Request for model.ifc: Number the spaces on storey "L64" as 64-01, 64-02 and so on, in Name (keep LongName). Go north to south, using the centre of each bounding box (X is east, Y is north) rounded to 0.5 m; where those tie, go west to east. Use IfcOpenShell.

First a look at what the model holds.

```python
import ifcopenshell
import ifcopenshell.util.element
import ifcopenshell.util.placement

model = ifcopenshell.open("model.ifc")
print(model.schema)
storey = next(s for s in model.by_type("IfcBuildingStorey") if s.Name == "L64")
spaces = [e for e in ifcopenshell.util.element.get_decomposition(storey) if e.is_a("IfcSpace")]
for e in sorted(spaces, key=lambda e: e.id()):
    origin = ifcopenshell.util.placement.get_local_placement(e.ObjectPlacement)[:3, 3]
    print(e.id(), e.Name, e.LongName, origin.round(2) + 0.0, sep=" | ")
```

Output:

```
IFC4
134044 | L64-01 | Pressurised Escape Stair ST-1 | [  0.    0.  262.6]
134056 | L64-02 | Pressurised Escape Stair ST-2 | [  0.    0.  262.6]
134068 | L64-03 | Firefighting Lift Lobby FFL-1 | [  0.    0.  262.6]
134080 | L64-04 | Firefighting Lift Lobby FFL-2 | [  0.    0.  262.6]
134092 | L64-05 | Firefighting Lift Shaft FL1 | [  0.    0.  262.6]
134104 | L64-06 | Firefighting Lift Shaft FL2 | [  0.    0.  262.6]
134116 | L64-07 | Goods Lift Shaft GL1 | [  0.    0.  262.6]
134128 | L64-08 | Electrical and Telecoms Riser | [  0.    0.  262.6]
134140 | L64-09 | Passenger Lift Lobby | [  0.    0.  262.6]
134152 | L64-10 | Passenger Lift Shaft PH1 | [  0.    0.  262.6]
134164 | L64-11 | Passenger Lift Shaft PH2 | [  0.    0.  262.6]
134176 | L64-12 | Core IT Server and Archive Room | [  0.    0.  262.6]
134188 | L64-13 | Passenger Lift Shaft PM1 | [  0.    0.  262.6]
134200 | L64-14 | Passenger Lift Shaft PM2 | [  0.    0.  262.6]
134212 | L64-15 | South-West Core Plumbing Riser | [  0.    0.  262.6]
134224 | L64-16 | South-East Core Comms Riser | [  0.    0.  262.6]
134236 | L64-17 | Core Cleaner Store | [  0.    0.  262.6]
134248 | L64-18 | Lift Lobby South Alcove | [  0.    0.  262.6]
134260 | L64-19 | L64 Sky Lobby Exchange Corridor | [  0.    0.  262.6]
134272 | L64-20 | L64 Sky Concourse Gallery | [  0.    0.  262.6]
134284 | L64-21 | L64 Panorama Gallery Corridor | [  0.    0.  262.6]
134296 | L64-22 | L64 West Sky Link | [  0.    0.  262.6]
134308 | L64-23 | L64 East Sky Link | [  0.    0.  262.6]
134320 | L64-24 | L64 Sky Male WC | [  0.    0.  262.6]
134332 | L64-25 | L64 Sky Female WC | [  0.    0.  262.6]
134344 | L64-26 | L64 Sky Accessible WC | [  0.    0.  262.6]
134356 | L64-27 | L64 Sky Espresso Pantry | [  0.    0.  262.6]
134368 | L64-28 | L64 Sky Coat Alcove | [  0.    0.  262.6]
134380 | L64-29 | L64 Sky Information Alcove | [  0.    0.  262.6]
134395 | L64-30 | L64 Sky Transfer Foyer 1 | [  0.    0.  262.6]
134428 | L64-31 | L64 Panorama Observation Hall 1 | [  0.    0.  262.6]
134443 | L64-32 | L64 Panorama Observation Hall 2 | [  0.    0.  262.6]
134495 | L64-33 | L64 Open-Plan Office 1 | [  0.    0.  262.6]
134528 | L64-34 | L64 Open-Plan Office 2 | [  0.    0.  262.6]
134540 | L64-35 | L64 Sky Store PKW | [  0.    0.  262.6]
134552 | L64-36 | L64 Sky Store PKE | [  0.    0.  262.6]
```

```python
import ifcopenshell
import ifcopenshell.geom
import ifcopenshell.util.element
import ifcopenshell.util.shape

model = ifcopenshell.open("model.ifc")
settings = ifcopenshell.geom.settings()
settings.set("use-world-coords", True)


def centre(element):
    shape = ifcopenshell.geom.create_shape(settings, element)
    return ifcopenshell.util.shape.get_bbox_centroid(shape.geometry)


storey = next(s for s in model.by_type("IfcBuildingStorey") if s.Name == "L64")
spaces = [e for e in ifcopenshell.util.element.get_decomposition(storey) if e.is_a("IfcSpace")]

# Insertion points can sit at a corner or the storey origin, so sort by the geometry (in metres).
centres = {e: centre(e) for e in spaces}
spaces.sort(key=lambda e: (-round(centres[e][1] / 0.5), centres[e][0]))

for i, e in enumerate(spaces, start=1):
    number = f"64-{i:02d}"
    e.Name = number
    print(e.id(), number)

model.write("model_updated.ifc")
```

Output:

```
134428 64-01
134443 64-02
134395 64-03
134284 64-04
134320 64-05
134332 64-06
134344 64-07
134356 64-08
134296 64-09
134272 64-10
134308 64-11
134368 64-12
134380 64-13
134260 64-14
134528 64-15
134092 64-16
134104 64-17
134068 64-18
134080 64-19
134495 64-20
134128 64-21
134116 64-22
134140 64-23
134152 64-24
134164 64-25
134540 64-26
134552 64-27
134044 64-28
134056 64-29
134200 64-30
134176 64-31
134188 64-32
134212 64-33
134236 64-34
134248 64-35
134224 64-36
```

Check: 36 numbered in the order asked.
